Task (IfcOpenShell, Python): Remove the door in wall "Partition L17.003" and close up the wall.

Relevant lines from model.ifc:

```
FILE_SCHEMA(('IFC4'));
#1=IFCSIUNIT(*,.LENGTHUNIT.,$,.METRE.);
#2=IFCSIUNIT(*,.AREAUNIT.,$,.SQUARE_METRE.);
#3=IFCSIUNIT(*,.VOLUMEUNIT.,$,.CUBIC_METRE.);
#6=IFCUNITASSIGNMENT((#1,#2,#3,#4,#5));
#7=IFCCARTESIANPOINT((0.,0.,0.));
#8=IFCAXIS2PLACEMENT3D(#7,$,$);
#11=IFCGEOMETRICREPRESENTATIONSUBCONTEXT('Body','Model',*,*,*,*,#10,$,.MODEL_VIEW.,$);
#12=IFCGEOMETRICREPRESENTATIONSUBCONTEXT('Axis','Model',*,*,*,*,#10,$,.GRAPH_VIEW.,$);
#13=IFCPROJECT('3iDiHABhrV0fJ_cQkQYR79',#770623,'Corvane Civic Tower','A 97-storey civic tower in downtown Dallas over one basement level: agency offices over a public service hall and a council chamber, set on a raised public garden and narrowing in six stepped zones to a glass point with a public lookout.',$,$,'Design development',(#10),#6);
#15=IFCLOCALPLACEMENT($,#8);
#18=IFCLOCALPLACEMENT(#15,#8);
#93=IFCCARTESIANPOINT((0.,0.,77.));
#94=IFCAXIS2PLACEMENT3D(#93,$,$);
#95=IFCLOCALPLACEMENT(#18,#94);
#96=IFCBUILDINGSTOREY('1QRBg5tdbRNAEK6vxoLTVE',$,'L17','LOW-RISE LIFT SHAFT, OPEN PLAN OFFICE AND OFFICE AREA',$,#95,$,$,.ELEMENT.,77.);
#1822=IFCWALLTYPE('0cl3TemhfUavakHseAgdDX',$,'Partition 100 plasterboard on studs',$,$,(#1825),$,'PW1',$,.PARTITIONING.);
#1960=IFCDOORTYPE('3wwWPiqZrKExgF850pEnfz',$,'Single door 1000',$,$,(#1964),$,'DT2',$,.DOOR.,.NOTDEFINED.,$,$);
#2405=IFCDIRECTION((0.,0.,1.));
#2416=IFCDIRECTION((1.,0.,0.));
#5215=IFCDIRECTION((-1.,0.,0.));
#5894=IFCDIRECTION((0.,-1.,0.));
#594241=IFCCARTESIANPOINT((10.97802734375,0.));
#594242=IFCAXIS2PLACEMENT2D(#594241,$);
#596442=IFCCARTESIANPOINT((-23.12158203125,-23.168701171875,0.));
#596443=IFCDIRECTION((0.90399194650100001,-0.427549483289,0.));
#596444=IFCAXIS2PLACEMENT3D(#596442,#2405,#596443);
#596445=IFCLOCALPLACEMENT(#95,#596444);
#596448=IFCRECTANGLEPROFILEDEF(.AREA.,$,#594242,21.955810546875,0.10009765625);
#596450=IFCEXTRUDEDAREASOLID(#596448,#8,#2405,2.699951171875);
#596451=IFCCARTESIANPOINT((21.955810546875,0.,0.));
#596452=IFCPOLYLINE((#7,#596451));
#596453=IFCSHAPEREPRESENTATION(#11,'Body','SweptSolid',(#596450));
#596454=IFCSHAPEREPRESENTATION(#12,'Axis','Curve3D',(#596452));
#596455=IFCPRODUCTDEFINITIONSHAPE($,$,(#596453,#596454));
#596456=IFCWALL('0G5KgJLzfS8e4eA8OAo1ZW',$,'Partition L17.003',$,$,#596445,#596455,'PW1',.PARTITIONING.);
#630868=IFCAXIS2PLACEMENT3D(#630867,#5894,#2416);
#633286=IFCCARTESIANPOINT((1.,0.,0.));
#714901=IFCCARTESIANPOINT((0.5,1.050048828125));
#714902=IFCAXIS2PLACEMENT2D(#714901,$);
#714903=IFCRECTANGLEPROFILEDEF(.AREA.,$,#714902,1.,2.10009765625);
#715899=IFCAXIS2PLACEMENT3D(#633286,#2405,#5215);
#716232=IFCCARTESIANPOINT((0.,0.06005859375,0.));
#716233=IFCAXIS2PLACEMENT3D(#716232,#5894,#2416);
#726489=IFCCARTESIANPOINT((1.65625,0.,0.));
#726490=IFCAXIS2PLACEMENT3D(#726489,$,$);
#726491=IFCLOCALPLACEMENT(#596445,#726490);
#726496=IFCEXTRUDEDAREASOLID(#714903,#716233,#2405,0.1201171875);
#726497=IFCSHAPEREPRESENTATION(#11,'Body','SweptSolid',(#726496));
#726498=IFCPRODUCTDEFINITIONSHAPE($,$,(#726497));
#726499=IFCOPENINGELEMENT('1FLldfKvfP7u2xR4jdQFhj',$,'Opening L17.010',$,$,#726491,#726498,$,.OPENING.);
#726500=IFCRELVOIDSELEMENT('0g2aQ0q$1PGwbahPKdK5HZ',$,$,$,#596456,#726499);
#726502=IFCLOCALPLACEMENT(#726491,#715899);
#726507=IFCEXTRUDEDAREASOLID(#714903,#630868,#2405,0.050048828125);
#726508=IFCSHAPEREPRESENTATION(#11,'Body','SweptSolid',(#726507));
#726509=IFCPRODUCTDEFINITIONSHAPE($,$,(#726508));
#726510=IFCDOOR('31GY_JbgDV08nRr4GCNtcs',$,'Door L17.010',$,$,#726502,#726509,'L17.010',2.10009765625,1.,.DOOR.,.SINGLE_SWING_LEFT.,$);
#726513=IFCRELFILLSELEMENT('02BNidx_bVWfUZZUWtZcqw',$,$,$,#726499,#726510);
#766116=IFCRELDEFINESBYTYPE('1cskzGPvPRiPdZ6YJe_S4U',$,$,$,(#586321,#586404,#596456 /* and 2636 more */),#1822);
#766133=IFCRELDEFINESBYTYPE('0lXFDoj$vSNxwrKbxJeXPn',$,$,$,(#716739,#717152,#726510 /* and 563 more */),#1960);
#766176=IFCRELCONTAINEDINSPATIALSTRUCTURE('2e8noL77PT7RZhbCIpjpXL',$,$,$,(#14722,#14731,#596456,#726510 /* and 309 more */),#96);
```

```python
import ifcopenshell
import ifcopenshell.api.feature
import ifcopenshell.api.root
import ifcopenshell.geom
import ifcopenshell.util.shape

model = ifcopenshell.open("model.ifc")
settings = ifcopenshell.geom.settings()


def volume(element):
    """Net volume in cubic metres, openings subtracted."""
    shape = ifcopenshell.geom.create_shape(settings, element)
    return ifcopenshell.util.shape.get_volume(shape.geometry)


door = model.by_guid("31GY_JbgDV08nRr4GCNtcs")
opening = door.FillsVoids[0].RelatingOpeningElement
wall = opening.VoidsElements[0].RelatingBuildingElement
before = volume(wall)

ifcopenshell.api.root.remove_product(model, product=door)
ifcopenshell.api.feature.remove_feature(model, feature=opening)

after = volume(wall)

print(f"wall volume {before:.3f} -> {after:.3f} m3")

model.write("model_rev.ifc")
```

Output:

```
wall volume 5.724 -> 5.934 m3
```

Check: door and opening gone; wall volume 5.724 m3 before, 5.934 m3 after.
